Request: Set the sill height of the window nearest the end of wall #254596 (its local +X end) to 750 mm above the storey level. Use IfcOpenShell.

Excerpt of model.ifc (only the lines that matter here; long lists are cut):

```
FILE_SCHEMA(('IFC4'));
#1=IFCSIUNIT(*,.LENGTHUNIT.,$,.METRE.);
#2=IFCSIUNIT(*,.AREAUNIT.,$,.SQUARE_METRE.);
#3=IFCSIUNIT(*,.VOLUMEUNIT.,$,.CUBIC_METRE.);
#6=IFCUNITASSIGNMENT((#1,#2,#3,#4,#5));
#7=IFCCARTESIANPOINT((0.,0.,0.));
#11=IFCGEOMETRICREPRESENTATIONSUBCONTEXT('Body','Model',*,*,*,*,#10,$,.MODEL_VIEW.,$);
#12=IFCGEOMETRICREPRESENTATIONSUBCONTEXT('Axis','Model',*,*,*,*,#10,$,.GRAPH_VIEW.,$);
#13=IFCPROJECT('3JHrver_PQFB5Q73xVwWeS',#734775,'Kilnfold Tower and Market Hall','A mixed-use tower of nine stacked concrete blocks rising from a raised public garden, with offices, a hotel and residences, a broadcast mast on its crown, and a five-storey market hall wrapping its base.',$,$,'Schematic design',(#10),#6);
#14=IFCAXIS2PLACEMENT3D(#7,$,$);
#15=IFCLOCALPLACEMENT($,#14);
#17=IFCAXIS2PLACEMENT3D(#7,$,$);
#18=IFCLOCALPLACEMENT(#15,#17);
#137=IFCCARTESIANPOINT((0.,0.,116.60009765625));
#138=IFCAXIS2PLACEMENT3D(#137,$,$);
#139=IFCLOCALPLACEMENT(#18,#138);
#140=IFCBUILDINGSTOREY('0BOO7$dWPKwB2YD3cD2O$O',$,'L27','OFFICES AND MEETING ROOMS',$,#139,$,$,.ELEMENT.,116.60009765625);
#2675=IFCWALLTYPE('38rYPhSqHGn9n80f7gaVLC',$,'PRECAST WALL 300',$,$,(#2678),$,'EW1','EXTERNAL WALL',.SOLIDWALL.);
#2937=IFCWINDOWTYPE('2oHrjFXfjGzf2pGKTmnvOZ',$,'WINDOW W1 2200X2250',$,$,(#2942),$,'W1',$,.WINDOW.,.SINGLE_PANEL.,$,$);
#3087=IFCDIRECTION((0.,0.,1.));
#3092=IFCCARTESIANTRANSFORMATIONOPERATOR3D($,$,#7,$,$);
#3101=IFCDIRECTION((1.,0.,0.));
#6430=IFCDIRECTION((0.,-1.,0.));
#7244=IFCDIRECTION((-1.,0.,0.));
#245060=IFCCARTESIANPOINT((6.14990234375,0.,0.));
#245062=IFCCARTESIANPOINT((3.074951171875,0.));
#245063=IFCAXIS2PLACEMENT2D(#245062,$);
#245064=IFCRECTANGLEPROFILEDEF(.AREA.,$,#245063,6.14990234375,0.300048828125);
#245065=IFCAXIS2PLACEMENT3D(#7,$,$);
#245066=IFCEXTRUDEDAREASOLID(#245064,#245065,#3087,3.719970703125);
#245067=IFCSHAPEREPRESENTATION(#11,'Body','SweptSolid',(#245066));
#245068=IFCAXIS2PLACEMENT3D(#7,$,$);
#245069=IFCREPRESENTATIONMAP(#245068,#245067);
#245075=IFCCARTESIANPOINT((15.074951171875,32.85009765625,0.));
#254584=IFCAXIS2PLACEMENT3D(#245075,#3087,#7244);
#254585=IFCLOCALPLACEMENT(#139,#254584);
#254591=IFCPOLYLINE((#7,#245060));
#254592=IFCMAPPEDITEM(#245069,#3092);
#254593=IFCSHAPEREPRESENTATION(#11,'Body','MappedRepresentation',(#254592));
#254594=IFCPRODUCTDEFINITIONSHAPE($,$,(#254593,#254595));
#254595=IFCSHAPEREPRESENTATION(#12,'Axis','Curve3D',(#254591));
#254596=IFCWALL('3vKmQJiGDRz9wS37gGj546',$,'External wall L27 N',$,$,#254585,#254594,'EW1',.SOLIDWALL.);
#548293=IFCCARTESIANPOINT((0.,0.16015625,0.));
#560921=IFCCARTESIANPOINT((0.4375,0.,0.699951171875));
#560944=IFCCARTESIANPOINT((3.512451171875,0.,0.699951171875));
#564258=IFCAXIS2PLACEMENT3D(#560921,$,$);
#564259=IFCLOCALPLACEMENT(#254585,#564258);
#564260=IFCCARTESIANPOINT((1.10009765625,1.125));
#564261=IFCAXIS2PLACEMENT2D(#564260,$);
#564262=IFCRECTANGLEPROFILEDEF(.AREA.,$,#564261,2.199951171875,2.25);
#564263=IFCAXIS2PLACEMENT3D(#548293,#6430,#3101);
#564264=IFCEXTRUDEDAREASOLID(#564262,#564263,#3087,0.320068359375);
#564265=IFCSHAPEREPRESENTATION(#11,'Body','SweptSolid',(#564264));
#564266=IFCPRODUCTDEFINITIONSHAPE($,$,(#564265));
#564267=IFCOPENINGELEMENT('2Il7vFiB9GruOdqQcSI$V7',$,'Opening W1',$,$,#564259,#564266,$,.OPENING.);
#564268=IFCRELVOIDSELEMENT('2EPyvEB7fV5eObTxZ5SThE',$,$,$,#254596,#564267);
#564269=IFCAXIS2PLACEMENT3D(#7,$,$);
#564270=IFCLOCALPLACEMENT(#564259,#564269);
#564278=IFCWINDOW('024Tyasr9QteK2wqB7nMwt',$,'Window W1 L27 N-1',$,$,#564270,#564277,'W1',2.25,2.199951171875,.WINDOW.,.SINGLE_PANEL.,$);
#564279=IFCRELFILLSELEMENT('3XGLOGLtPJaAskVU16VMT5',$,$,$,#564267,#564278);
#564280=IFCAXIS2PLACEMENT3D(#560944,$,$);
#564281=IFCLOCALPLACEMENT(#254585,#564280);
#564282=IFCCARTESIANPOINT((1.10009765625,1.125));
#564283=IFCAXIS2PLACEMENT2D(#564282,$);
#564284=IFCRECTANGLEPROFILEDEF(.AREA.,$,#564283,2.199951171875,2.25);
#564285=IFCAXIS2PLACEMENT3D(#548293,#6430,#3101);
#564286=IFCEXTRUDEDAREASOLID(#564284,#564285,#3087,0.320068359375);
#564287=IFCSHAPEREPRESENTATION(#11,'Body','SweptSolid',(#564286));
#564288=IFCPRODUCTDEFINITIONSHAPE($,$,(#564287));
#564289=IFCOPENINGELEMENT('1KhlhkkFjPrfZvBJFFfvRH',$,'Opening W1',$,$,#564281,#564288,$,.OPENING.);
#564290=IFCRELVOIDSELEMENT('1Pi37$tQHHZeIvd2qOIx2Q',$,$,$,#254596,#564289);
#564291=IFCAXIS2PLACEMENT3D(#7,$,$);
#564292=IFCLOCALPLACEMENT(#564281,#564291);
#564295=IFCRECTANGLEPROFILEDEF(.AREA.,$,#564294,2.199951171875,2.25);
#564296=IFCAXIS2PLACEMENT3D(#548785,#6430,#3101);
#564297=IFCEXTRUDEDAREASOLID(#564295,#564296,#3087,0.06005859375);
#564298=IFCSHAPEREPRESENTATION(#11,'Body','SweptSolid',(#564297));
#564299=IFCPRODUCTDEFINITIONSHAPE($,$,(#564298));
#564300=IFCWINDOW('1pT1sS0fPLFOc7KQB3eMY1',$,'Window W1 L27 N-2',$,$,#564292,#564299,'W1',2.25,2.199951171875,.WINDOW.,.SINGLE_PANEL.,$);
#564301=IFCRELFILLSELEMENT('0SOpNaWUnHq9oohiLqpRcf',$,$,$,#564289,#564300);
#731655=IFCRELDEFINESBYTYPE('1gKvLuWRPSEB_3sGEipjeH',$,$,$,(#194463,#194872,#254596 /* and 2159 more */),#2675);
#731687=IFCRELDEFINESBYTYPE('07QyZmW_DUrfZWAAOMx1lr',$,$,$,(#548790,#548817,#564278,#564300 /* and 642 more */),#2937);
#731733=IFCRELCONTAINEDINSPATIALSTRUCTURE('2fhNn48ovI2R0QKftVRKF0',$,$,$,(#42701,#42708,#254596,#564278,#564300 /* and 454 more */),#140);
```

```python
import numpy as np
import ifcopenshell
import ifcopenshell.api.geometry
import ifcopenshell.geom
import ifcopenshell.util.element
import ifcopenshell.util.placement
import ifcopenshell.util.shape
import ifcopenshell.util.unit

model = ifcopenshell.open("model.ifc")
unit_scale = ifcopenshell.util.unit.calculate_unit_scale(model)

window = model.by_id(564300)
opening = window.FillsVoids[0].RelatingOpeningElement
storey = ifcopenshell.util.element.get_container(window, ifc_class="IfcBuildingStorey")
level = ifcopenshell.util.placement.get_local_placement(storey.ObjectPlacement)[2, 3]

# The opening's origin need not be at the sill, so measure its lowest point.
shape = ifcopenshell.geom.create_shape(ifcopenshell.geom.settings(), opening)
bottom = ifcopenshell.util.shape.get_shape_bottom_elevation(shape, shape.geometry) / unit_scale
dz = level + 0.75 - bottom

shift = np.array([0.0, 0.0, dz])
# The window is placed relative to its opening, so it follows when the opening moves.
matrix = ifcopenshell.util.placement.get_local_placement(opening.ObjectPlacement)
matrix[:3, 3] += shift
ifcopenshell.api.geometry.edit_object_placement(
    model, product=opening, matrix=matrix, is_si=False, should_transform_children=True
)

print(f"moved by {dz * unit_scale:+.3f} m")

model.write("model_v2.ifc")
```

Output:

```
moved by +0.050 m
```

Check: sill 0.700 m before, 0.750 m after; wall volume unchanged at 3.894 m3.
